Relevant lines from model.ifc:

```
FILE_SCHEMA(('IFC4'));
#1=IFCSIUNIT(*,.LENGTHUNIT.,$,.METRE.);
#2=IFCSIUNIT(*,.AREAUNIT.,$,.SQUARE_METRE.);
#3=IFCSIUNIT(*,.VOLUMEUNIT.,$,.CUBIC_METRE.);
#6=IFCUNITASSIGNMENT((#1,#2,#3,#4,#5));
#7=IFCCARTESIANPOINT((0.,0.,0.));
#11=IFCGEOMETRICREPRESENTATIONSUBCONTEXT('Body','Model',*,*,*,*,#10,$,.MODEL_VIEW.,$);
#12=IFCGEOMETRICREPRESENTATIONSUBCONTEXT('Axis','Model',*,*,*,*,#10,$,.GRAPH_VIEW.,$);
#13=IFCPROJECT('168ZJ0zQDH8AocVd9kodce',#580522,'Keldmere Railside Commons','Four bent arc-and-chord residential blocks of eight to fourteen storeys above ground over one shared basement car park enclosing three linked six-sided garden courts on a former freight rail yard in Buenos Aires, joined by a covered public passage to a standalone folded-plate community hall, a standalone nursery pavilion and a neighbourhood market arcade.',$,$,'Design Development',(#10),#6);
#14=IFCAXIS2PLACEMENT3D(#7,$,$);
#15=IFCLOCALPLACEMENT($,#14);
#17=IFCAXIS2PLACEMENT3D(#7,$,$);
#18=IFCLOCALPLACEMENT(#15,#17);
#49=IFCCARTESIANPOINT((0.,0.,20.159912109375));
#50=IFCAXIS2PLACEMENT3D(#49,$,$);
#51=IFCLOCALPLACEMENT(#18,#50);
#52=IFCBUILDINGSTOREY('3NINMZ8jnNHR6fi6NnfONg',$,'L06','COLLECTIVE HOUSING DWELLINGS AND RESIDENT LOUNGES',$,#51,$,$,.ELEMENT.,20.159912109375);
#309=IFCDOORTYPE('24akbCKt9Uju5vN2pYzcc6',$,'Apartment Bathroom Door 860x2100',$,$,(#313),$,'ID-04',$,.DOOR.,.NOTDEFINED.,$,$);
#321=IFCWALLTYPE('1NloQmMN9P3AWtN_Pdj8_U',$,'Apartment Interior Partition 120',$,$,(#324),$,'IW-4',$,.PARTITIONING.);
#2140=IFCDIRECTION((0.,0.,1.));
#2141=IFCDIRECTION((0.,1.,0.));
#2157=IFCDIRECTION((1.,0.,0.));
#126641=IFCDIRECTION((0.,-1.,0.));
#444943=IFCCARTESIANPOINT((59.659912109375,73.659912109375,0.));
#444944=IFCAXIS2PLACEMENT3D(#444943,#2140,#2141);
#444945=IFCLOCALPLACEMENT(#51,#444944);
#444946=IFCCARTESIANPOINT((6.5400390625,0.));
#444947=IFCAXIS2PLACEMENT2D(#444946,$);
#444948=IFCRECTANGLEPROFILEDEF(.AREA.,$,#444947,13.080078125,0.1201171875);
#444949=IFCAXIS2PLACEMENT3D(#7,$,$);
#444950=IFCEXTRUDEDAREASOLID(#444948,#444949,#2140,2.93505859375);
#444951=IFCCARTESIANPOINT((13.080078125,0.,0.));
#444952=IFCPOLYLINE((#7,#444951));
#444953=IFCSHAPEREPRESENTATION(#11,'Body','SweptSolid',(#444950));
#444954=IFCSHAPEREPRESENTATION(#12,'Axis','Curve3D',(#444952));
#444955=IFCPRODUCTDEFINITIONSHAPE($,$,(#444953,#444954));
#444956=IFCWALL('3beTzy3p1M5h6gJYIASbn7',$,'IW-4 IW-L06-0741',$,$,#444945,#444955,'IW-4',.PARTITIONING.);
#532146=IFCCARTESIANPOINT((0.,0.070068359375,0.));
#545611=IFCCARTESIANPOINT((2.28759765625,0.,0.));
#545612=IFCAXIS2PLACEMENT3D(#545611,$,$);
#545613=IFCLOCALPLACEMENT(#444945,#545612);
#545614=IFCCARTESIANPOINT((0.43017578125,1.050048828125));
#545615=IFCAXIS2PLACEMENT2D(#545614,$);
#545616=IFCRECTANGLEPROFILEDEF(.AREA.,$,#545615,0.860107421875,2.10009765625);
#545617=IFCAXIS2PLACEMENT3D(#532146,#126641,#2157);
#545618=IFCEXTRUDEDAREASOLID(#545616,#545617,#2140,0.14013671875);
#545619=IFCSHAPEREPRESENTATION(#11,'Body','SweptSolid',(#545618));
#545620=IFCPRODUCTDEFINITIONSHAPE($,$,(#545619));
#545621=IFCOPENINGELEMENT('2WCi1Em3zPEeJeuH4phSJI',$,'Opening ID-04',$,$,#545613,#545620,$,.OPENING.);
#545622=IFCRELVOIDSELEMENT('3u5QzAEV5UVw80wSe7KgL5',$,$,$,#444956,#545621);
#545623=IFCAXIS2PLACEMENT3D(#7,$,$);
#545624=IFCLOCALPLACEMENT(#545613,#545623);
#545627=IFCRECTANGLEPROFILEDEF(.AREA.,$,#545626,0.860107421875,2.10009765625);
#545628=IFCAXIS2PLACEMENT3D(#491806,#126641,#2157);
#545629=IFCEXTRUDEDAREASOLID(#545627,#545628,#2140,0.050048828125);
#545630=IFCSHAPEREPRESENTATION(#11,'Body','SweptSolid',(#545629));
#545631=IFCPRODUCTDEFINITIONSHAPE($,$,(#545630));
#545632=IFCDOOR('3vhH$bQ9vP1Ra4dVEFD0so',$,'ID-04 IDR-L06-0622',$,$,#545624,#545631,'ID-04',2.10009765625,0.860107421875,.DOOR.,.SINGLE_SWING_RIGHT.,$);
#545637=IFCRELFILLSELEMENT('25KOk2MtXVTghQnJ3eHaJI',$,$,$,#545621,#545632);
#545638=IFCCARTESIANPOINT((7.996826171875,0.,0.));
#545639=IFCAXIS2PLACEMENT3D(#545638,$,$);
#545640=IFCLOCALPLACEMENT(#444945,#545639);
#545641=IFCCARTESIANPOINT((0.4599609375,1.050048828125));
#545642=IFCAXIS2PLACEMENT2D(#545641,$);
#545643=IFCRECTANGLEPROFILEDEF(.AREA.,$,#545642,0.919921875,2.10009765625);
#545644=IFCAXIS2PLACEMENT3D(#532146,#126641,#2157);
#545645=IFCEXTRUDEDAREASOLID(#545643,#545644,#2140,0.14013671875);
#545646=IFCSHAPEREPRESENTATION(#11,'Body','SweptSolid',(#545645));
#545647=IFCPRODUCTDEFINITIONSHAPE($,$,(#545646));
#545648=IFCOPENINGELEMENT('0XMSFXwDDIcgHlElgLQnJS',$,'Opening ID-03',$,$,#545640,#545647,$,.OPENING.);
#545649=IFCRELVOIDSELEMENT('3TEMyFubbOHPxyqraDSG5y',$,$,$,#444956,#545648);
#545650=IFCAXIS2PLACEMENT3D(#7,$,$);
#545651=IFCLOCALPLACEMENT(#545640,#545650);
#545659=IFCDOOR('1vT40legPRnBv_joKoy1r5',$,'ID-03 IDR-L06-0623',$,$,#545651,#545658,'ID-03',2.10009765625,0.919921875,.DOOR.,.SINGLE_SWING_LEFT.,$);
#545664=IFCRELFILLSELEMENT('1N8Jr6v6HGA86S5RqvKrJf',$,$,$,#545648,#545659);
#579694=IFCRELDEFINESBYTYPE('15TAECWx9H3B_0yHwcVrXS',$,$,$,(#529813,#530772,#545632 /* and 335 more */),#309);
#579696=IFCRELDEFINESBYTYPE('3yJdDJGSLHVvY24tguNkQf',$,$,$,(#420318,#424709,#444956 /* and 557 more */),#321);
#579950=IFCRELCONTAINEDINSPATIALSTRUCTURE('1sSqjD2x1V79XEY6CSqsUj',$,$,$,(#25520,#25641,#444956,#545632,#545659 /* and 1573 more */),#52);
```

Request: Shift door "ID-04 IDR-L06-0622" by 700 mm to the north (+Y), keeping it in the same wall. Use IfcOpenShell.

```python
import ifcopenshell
import ifcopenshell.api.geometry
import ifcopenshell.util.placement
import ifcopenshell.util.unit

model = ifcopenshell.open("model.ifc")
unit_scale = ifcopenshell.util.unit.calculate_unit_scale(model)

door = model.by_id(545632)
opening = door.FillsVoids[0].RelatingOpeningElement
wall = opening.VoidsElements[0].RelatingBuildingElement

wall_matrix = ifcopenshell.util.placement.get_local_placement(wall.ObjectPlacement)
shift = wall_matrix[:3, 0] * 0.7 / unit_scale
before = ifcopenshell.util.placement.get_local_placement(door.ObjectPlacement)[:3, 3].copy()

# The door is placed relative to its opening, so it follows when the opening moves.
matrix = ifcopenshell.util.placement.get_local_placement(opening.ObjectPlacement)
matrix[:3, 3] += shift
ifcopenshell.api.geometry.edit_object_placement(
    model, product=opening, matrix=matrix, is_si=False, should_transform_children=True
)

after = ifcopenshell.util.placement.get_local_placement(door.ObjectPlacement)[:3, 3]
print("door moved by", (after - before).round(3) + 0.0)

model.write("model_v2.ifc")
```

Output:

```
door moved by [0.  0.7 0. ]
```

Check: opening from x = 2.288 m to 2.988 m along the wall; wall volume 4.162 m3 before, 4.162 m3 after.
